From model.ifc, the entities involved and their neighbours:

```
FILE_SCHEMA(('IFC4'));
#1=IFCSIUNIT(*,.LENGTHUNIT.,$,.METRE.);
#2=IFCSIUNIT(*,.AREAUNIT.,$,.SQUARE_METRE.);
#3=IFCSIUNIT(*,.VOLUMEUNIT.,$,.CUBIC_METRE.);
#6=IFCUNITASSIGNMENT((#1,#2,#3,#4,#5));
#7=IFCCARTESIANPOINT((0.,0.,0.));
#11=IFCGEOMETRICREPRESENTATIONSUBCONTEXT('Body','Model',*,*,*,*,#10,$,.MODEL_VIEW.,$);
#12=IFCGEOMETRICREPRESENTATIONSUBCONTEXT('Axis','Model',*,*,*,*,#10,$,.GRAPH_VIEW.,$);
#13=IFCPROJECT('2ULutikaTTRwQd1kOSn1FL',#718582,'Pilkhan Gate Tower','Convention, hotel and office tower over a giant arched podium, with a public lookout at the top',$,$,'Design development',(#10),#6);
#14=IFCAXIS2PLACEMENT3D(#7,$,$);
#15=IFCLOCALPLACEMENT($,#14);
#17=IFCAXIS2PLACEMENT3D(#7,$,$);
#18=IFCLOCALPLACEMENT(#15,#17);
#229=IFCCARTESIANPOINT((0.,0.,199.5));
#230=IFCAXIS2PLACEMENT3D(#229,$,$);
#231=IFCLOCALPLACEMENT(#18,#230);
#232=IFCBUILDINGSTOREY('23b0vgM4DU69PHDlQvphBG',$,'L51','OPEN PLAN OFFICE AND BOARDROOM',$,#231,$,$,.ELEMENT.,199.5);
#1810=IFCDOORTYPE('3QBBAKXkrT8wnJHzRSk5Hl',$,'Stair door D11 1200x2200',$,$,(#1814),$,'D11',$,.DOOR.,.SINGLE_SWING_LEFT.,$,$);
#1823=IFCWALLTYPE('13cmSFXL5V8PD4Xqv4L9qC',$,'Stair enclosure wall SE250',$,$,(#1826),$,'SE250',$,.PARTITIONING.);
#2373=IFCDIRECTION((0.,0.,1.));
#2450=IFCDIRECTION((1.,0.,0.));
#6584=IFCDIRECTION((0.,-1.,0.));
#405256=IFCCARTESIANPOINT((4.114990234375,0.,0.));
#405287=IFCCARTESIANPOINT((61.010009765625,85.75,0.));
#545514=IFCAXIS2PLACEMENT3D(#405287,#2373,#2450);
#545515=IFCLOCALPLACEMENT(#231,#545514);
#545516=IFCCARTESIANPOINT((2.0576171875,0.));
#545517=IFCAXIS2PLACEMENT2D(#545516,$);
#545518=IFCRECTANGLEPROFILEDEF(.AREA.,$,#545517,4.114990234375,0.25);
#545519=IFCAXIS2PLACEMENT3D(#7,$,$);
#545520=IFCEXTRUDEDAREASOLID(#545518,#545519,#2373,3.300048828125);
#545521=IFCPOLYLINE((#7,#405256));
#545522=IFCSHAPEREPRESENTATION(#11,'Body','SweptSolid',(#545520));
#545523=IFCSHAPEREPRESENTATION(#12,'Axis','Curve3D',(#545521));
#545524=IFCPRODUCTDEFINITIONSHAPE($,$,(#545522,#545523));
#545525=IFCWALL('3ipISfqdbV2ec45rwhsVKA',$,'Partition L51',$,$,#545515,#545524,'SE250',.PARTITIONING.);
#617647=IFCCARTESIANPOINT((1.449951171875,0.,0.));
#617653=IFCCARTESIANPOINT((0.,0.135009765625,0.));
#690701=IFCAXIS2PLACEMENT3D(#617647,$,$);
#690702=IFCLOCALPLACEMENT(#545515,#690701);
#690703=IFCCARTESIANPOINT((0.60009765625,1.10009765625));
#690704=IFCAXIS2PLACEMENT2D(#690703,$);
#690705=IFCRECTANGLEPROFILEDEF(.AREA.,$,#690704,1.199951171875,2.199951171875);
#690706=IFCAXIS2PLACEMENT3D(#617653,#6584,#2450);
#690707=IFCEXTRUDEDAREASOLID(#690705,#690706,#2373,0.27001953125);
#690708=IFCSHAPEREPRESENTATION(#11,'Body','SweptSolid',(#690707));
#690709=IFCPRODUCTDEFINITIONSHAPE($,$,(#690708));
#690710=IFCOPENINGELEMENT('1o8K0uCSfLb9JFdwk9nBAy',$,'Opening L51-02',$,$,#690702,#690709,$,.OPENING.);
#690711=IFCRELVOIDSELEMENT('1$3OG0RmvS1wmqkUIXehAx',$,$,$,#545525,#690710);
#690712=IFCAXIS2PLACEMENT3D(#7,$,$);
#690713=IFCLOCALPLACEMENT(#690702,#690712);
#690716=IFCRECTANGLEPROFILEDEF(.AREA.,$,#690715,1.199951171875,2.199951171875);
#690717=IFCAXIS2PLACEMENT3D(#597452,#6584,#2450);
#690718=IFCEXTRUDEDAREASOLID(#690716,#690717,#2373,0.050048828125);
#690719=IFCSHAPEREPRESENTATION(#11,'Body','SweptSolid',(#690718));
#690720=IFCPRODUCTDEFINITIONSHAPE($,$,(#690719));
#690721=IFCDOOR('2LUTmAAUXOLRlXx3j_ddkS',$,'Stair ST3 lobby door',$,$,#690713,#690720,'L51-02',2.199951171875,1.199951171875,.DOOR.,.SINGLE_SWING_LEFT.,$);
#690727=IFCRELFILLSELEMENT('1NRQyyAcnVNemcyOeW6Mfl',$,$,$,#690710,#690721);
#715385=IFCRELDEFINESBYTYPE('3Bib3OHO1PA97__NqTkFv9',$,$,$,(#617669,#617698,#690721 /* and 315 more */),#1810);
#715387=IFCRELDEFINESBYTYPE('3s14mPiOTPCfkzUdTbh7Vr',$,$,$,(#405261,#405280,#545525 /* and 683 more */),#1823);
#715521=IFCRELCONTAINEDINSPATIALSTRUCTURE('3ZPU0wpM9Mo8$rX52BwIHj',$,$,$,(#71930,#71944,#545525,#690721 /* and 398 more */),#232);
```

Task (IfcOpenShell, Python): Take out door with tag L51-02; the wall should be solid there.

```python
import ifcopenshell
import ifcopenshell.api.feature
import ifcopenshell.api.root
import ifcopenshell.geom
import ifcopenshell.util.shape

model = ifcopenshell.open("model.ifc")
settings = ifcopenshell.geom.settings()


def volume(element):
    """Net volume in cubic metres, openings subtracted."""
    shape = ifcopenshell.geom.create_shape(settings, element)
    return ifcopenshell.util.shape.get_volume(shape.geometry)


door = model.by_id(690721)
opening = door.FillsVoids[0].RelatingOpeningElement
wall = opening.VoidsElements[0].RelatingBuildingElement
before = volume(wall)

ifcopenshell.api.root.remove_product(model, product=door)
ifcopenshell.api.feature.remove_feature(model, feature=opening)

after = volume(wall)

print(f"wall volume {before:.3f} -> {after:.3f} m3")

model.write("model-out.ifc")
```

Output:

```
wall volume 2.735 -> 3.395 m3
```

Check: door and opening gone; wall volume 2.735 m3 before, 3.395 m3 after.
